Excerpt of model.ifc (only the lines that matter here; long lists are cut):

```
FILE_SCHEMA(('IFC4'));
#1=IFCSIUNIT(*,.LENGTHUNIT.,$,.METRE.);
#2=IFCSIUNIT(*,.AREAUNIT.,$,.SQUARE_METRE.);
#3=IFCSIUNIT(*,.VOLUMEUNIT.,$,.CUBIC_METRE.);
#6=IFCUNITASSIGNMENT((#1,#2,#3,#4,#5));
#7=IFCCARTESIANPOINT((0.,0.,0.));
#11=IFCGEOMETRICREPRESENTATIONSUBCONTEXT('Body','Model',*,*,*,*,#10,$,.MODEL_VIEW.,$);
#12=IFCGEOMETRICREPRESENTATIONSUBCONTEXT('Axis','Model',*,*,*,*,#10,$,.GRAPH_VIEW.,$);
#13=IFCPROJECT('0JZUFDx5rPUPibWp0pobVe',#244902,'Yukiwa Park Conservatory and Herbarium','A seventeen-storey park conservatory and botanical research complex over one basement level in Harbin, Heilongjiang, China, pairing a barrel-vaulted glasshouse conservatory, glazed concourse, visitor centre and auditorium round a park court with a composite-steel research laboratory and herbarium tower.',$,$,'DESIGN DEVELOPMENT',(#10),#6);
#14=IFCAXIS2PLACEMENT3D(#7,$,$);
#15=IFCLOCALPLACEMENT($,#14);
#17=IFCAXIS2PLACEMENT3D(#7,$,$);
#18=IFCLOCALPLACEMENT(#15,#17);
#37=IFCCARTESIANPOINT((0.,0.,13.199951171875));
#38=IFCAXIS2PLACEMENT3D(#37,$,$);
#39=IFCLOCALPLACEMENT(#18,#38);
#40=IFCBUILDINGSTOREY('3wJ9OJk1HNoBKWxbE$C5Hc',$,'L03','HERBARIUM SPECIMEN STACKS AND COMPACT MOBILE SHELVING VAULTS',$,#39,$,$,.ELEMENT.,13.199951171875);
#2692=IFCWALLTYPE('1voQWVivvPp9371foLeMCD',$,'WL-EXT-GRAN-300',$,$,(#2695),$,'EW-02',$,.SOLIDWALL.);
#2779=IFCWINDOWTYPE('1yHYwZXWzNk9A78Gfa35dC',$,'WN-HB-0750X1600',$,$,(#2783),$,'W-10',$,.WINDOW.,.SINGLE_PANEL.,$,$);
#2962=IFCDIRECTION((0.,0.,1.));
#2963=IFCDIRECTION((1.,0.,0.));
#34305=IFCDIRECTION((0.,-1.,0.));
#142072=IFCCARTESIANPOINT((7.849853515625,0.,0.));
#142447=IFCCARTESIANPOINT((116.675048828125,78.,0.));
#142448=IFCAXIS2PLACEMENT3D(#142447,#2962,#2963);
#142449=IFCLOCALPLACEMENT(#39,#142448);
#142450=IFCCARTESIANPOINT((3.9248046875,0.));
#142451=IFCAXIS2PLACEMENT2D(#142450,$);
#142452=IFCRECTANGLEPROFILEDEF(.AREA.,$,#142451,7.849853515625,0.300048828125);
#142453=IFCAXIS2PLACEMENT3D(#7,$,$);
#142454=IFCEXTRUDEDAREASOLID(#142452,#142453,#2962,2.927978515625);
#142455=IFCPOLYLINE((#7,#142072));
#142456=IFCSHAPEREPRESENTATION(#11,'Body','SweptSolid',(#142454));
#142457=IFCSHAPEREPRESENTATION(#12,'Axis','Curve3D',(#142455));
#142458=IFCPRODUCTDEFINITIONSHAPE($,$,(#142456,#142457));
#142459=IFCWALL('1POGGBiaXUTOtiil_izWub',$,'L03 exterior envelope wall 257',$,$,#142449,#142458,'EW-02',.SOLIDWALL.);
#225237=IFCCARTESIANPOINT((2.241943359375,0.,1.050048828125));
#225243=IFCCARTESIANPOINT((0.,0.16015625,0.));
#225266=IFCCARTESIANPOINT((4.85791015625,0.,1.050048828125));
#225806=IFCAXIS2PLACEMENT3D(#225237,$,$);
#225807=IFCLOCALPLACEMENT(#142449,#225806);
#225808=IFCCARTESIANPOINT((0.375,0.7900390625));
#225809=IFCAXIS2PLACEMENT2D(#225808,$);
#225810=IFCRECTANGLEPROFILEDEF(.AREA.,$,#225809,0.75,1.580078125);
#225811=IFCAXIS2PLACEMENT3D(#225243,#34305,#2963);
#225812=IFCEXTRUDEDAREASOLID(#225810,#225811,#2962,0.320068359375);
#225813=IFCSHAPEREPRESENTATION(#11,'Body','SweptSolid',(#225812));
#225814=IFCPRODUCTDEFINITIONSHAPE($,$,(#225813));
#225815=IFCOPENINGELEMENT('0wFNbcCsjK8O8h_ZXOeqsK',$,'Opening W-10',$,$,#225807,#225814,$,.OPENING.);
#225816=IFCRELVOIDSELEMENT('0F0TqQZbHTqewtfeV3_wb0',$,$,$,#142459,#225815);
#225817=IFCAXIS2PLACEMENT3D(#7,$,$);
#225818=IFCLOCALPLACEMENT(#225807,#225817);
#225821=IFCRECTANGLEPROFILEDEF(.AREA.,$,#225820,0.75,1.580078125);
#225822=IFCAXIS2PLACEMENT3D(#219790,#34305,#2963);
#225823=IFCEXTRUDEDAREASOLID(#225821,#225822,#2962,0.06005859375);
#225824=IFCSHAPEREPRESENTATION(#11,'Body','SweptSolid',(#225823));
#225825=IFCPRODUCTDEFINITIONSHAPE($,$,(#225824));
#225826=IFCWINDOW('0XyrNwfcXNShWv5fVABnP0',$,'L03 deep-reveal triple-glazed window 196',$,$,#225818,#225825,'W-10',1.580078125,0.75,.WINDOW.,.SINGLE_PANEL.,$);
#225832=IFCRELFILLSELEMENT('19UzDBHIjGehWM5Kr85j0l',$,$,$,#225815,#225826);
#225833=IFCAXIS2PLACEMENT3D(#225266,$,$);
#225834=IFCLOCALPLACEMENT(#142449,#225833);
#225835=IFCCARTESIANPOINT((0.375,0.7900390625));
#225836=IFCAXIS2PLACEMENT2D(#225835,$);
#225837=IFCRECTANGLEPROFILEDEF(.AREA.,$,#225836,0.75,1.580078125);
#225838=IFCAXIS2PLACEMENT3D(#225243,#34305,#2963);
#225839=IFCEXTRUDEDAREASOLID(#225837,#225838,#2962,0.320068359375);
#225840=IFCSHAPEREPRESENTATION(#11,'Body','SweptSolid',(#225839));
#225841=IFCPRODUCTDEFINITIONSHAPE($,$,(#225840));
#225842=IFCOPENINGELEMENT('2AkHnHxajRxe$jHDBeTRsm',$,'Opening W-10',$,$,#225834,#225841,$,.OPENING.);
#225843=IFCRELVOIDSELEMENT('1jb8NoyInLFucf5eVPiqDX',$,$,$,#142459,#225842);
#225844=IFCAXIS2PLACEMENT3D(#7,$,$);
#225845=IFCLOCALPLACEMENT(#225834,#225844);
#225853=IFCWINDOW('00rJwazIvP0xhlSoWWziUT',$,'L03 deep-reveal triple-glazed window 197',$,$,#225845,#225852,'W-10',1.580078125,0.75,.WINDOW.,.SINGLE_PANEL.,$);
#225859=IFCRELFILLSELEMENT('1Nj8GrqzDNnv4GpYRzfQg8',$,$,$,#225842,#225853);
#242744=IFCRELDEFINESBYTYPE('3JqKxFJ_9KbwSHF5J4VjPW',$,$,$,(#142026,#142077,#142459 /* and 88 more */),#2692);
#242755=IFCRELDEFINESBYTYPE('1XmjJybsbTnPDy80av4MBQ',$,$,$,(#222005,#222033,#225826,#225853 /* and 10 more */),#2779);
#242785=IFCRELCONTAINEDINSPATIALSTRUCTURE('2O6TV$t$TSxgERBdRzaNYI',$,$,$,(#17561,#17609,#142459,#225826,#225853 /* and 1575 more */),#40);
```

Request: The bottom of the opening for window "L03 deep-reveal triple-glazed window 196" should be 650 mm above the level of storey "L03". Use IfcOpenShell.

```python
import numpy as np
import ifcopenshell
import ifcopenshell.api.geometry
import ifcopenshell.geom
import ifcopenshell.util.element
import ifcopenshell.util.placement
import ifcopenshell.util.shape
import ifcopenshell.util.unit

model = ifcopenshell.open("model.ifc")
unit_scale = ifcopenshell.util.unit.calculate_unit_scale(model)

window = model.by_id(225826)
opening = window.FillsVoids[0].RelatingOpeningElement
storey = ifcopenshell.util.element.get_container(window, ifc_class="IfcBuildingStorey")
level = ifcopenshell.util.placement.get_local_placement(storey.ObjectPlacement)[2, 3]

# The opening's origin need not be at the sill, so measure its lowest point.
shape = ifcopenshell.geom.create_shape(ifcopenshell.geom.settings(), opening)
bottom = ifcopenshell.util.shape.get_shape_bottom_elevation(shape, shape.geometry) / unit_scale
dz = level + 0.65 - bottom

shift = np.array([0.0, 0.0, dz])
# The window is placed relative to its opening, so it follows when the opening moves.
matrix = ifcopenshell.util.placement.get_local_placement(opening.ObjectPlacement)
matrix[:3, 3] += shift
ifcopenshell.api.geometry.edit_object_placement(
    model, product=opening, matrix=matrix, is_si=False, should_transform_children=True
)

print(f"moved by {dz * unit_scale:+.3f} m")

model.write("model-out.ifc")
```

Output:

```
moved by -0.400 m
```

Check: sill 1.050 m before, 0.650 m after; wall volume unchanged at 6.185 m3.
